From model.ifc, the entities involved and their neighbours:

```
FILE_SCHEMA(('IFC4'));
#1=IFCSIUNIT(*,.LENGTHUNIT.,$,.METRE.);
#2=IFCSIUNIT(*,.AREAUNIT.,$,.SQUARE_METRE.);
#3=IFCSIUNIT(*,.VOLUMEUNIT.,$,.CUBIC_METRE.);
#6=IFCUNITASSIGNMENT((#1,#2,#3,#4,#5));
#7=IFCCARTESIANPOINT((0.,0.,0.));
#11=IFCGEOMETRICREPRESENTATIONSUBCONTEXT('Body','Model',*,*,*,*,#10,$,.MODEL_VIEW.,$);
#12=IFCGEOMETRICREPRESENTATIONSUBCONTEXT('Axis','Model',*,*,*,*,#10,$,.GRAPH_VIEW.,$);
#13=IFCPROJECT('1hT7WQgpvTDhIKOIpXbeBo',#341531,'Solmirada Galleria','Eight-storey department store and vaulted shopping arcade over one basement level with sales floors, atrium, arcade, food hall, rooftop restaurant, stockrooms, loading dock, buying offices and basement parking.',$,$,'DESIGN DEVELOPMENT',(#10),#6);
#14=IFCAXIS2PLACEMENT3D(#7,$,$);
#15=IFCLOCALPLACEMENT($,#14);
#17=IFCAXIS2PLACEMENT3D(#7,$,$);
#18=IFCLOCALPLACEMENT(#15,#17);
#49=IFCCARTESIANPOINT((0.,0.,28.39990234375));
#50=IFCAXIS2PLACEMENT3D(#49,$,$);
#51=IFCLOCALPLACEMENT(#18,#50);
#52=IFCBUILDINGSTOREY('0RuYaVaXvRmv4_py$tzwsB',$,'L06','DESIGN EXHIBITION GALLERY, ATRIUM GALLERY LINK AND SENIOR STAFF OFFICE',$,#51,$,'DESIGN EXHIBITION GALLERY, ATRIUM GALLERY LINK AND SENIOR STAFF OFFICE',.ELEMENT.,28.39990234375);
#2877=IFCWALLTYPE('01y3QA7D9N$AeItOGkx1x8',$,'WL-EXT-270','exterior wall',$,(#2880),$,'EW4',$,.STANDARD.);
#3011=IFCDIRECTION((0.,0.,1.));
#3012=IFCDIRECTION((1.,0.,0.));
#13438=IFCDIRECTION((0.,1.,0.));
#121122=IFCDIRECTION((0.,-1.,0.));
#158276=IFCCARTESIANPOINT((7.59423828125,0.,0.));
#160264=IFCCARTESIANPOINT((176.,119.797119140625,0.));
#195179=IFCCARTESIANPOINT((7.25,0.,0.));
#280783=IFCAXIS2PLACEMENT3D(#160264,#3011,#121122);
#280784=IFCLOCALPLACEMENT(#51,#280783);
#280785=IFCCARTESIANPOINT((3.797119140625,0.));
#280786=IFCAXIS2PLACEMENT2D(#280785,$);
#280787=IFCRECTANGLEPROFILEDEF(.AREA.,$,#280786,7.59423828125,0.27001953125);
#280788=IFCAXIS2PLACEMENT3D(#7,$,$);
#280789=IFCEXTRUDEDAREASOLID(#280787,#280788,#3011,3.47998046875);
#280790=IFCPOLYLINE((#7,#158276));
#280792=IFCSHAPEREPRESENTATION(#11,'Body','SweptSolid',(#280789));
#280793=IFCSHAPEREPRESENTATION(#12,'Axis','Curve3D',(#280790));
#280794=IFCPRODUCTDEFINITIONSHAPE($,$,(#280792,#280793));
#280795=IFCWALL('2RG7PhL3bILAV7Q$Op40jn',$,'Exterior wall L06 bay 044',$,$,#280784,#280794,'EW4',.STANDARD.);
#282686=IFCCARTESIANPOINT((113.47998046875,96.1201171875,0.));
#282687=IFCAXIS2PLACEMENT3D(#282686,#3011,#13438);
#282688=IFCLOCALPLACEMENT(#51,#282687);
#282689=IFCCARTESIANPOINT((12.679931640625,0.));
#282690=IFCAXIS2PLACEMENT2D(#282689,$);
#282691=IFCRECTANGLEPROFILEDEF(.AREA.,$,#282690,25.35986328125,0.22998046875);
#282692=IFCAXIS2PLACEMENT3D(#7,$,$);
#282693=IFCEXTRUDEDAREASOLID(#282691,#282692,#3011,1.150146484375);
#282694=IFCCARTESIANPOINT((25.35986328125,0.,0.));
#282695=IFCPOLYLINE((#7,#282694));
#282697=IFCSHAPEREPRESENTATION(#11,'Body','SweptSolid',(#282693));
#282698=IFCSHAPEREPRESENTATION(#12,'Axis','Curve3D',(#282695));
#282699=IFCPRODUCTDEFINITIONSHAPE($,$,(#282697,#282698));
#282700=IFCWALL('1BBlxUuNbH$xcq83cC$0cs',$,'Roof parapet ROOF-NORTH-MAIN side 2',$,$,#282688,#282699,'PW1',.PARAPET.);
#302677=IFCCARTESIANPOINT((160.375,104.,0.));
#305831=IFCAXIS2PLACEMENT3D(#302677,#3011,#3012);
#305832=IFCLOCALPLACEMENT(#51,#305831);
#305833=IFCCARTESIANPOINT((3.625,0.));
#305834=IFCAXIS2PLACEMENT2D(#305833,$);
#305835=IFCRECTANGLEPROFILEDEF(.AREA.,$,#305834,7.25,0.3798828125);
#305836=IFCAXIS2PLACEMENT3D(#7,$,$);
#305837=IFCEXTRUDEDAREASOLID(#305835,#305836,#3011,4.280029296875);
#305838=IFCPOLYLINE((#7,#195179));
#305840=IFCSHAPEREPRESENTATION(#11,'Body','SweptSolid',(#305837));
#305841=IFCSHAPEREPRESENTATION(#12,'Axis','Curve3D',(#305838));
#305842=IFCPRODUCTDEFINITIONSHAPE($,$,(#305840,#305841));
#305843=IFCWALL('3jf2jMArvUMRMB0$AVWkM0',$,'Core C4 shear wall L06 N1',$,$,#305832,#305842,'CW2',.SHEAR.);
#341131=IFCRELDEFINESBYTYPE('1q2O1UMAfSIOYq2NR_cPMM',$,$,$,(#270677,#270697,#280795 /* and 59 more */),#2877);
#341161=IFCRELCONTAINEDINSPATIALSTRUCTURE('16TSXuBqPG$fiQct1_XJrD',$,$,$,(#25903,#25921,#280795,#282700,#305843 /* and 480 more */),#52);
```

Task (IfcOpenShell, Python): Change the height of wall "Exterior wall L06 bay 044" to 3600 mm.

```python
import ifcopenshell
import ifcopenshell.geom
import ifcopenshell.util.representation
import ifcopenshell.util.shape
import ifcopenshell.util.unit

model = ifcopenshell.open("model.ifc")
unit_scale = ifcopenshell.util.unit.calculate_unit_scale(model)
settings = ifcopenshell.geom.settings()


def volume(element):
    """Net volume in cubic metres, openings subtracted."""
    shape = ifcopenshell.geom.create_shape(settings, element)
    return ifcopenshell.util.shape.get_volume(shape.geometry)


wall = model.by_guid("2RG7PhL3bILAV7Q$Op40jn")
before = volume(wall)

body = ifcopenshell.util.representation.get_representation(wall, "Model", "Body")
solid = body.Items[0]
old_height = solid.Depth
solid.Depth = 3.6 / unit_scale
after = volume(wall)

print(f"height {old_height:g} -> {solid.Depth:g}, volume {before:.3f} -> {after:.3f} m3")

model.write("model_updated.ifc")
```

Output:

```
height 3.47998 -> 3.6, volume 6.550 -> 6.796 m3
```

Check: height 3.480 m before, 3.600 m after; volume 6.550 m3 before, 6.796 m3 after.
